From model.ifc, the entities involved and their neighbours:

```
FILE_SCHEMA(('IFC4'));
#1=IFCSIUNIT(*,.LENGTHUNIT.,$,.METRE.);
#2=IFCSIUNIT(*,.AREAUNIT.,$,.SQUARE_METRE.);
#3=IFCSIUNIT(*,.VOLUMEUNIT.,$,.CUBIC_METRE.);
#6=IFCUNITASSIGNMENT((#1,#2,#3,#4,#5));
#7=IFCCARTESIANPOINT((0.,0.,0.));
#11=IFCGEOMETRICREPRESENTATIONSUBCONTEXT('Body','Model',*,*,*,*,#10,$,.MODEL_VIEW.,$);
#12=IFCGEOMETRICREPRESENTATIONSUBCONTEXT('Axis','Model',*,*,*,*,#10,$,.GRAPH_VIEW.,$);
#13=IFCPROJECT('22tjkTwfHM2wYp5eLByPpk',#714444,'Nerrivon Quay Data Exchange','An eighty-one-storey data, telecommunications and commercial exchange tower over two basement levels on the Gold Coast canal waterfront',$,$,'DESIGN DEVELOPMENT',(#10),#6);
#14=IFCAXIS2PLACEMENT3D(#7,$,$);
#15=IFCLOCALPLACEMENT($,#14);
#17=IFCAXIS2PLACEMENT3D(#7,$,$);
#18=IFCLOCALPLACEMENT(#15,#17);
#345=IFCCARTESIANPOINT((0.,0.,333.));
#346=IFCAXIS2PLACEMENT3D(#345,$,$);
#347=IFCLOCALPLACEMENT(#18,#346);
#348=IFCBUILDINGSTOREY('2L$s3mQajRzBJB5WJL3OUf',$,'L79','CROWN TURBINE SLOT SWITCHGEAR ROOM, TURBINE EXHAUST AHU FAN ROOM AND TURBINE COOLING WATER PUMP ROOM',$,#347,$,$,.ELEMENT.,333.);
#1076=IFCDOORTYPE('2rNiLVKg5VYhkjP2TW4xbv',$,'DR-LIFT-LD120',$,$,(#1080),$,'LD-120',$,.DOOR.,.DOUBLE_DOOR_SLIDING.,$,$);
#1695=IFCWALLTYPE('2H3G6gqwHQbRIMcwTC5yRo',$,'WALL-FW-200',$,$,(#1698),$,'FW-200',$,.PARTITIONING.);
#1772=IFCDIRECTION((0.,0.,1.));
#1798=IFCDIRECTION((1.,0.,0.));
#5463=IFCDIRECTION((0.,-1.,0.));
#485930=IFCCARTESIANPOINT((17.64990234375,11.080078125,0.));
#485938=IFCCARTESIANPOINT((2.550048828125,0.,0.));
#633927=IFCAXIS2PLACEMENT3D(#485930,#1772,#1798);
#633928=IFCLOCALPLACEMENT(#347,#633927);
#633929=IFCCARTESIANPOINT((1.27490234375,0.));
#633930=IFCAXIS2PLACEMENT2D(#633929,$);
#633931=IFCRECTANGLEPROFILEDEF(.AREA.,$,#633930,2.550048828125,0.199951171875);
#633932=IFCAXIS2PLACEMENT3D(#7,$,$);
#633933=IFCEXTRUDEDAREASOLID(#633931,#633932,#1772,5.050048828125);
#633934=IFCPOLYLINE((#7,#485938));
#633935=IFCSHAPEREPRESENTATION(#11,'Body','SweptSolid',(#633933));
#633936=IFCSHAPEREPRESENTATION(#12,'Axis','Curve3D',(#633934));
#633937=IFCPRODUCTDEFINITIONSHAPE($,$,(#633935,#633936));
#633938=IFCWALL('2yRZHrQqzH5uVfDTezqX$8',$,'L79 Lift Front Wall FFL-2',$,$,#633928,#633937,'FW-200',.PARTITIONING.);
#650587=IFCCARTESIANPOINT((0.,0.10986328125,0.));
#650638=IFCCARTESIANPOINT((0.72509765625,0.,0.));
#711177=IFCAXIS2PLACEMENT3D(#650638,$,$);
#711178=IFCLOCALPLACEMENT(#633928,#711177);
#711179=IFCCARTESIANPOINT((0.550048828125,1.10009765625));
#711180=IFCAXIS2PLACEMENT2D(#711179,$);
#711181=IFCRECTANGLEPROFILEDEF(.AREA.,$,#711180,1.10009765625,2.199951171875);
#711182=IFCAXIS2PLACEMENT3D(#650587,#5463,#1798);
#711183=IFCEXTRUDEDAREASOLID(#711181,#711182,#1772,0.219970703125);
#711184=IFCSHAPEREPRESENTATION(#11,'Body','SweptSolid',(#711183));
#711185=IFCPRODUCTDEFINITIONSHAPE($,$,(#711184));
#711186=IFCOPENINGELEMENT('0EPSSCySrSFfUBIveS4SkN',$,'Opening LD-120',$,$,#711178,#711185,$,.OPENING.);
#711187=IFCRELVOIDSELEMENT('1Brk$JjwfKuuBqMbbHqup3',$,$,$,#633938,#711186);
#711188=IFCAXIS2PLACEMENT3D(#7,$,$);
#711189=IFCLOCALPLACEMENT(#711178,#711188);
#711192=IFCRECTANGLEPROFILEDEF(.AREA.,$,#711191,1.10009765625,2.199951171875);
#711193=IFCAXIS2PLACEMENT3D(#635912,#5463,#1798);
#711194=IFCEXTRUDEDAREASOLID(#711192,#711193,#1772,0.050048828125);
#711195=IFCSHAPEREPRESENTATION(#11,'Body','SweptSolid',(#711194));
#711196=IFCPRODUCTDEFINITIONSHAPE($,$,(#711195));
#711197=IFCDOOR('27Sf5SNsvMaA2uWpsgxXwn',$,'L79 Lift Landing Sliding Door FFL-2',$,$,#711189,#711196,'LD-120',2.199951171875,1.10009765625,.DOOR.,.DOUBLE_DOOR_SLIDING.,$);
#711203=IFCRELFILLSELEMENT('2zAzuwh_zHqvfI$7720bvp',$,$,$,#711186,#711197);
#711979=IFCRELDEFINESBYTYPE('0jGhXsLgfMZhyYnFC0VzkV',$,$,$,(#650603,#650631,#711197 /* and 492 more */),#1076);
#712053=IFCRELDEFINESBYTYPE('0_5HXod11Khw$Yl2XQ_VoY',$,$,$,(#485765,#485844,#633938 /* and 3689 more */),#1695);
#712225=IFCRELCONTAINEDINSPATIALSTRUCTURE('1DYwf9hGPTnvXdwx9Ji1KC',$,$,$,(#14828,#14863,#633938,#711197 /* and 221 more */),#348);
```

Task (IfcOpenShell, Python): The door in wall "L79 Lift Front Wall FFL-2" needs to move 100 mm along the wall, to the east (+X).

```python
import ifcopenshell
import ifcopenshell.api.geometry
import ifcopenshell.util.placement
import ifcopenshell.util.unit

model = ifcopenshell.open("model.ifc")
unit_scale = ifcopenshell.util.unit.calculate_unit_scale(model)

door = model.by_guid("27Sf5SNsvMaA2uWpsgxXwn")
opening = door.FillsVoids[0].RelatingOpeningElement
wall = opening.VoidsElements[0].RelatingBuildingElement

wall_matrix = ifcopenshell.util.placement.get_local_placement(wall.ObjectPlacement)
shift = wall_matrix[:3, 0] * 0.1 / unit_scale
before = ifcopenshell.util.placement.get_local_placement(door.ObjectPlacement)[:3, 3].copy()

# The door is placed relative to its opening, so it follows when the opening moves.
matrix = ifcopenshell.util.placement.get_local_placement(opening.ObjectPlacement)
matrix[:3, 3] += shift
ifcopenshell.api.geometry.edit_object_placement(
    model, product=opening, matrix=matrix, is_si=False, should_transform_children=True
)

after = ifcopenshell.util.placement.get_local_placement(door.ObjectPlacement)[:3, 3]
print("door moved by", (after - before).round(3) + 0.0)

model.write("model_updated.ifc")
```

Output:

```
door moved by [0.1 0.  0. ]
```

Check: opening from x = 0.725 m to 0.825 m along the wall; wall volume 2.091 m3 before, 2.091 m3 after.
